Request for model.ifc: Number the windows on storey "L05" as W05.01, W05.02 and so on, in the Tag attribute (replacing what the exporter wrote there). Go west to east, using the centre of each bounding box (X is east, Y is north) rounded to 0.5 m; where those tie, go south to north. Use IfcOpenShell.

First a look at what the model holds.

```python
import ifcopenshell
import ifcopenshell.util.element
import ifcopenshell.util.placement

model = ifcopenshell.open("model.ifc")
print(model.schema)
storey = next(s for s in model.by_type("IfcBuildingStorey") if s.Name == "L05")
windows = [e for e in ifcopenshell.util.element.get_decomposition(storey) if e.is_a("IfcWindow")]
for e in sorted(windows, key=lambda e: e.id()):
    origin = ifcopenshell.util.placement.get_local_placement(e.ObjectPlacement)[:3, 3]
    print(e.id(), e.Tag, e.Name, origin.round(2) + 0.0, sep=" | ")
```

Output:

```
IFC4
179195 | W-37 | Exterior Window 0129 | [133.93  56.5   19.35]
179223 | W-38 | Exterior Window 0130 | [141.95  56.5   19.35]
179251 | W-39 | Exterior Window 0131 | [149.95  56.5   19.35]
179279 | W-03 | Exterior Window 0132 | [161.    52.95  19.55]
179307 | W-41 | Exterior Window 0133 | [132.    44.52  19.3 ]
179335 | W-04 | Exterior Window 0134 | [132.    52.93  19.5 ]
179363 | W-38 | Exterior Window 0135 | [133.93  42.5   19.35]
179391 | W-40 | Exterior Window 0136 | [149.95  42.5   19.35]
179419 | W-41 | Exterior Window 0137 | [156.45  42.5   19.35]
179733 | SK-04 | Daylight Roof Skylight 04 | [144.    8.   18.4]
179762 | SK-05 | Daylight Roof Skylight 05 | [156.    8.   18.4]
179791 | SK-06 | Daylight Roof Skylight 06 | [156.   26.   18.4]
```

```python
import ifcopenshell
import ifcopenshell.geom
import ifcopenshell.util.element
import ifcopenshell.util.shape

model = ifcopenshell.open("model.ifc")
settings = ifcopenshell.geom.settings()
settings.set("use-world-coords", True)


def centre(element):
    shape = ifcopenshell.geom.create_shape(settings, element)
    return ifcopenshell.util.shape.get_bbox_centroid(shape.geometry)


storey = next(s for s in model.by_type("IfcBuildingStorey") if s.Name == "L05")
windows = [e for e in ifcopenshell.util.element.get_decomposition(storey) if e.is_a("IfcWindow")]

# Insertion points can sit at a corner or the storey origin, so sort by the geometry (in metres).
centres = {e: centre(e) for e in windows}
windows.sort(key=lambda e: (round(centres[e][0] / 0.5), centres[e][1]))

for i, e in enumerate(windows, start=1):
    number = f"W05.{i:02d}"
    e.Tag = number
    print(e.id(), number)

model.write("model_rev.ifc")
```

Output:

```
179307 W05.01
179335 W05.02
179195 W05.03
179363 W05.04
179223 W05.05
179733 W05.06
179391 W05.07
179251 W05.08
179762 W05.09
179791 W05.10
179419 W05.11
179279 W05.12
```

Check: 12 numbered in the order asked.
